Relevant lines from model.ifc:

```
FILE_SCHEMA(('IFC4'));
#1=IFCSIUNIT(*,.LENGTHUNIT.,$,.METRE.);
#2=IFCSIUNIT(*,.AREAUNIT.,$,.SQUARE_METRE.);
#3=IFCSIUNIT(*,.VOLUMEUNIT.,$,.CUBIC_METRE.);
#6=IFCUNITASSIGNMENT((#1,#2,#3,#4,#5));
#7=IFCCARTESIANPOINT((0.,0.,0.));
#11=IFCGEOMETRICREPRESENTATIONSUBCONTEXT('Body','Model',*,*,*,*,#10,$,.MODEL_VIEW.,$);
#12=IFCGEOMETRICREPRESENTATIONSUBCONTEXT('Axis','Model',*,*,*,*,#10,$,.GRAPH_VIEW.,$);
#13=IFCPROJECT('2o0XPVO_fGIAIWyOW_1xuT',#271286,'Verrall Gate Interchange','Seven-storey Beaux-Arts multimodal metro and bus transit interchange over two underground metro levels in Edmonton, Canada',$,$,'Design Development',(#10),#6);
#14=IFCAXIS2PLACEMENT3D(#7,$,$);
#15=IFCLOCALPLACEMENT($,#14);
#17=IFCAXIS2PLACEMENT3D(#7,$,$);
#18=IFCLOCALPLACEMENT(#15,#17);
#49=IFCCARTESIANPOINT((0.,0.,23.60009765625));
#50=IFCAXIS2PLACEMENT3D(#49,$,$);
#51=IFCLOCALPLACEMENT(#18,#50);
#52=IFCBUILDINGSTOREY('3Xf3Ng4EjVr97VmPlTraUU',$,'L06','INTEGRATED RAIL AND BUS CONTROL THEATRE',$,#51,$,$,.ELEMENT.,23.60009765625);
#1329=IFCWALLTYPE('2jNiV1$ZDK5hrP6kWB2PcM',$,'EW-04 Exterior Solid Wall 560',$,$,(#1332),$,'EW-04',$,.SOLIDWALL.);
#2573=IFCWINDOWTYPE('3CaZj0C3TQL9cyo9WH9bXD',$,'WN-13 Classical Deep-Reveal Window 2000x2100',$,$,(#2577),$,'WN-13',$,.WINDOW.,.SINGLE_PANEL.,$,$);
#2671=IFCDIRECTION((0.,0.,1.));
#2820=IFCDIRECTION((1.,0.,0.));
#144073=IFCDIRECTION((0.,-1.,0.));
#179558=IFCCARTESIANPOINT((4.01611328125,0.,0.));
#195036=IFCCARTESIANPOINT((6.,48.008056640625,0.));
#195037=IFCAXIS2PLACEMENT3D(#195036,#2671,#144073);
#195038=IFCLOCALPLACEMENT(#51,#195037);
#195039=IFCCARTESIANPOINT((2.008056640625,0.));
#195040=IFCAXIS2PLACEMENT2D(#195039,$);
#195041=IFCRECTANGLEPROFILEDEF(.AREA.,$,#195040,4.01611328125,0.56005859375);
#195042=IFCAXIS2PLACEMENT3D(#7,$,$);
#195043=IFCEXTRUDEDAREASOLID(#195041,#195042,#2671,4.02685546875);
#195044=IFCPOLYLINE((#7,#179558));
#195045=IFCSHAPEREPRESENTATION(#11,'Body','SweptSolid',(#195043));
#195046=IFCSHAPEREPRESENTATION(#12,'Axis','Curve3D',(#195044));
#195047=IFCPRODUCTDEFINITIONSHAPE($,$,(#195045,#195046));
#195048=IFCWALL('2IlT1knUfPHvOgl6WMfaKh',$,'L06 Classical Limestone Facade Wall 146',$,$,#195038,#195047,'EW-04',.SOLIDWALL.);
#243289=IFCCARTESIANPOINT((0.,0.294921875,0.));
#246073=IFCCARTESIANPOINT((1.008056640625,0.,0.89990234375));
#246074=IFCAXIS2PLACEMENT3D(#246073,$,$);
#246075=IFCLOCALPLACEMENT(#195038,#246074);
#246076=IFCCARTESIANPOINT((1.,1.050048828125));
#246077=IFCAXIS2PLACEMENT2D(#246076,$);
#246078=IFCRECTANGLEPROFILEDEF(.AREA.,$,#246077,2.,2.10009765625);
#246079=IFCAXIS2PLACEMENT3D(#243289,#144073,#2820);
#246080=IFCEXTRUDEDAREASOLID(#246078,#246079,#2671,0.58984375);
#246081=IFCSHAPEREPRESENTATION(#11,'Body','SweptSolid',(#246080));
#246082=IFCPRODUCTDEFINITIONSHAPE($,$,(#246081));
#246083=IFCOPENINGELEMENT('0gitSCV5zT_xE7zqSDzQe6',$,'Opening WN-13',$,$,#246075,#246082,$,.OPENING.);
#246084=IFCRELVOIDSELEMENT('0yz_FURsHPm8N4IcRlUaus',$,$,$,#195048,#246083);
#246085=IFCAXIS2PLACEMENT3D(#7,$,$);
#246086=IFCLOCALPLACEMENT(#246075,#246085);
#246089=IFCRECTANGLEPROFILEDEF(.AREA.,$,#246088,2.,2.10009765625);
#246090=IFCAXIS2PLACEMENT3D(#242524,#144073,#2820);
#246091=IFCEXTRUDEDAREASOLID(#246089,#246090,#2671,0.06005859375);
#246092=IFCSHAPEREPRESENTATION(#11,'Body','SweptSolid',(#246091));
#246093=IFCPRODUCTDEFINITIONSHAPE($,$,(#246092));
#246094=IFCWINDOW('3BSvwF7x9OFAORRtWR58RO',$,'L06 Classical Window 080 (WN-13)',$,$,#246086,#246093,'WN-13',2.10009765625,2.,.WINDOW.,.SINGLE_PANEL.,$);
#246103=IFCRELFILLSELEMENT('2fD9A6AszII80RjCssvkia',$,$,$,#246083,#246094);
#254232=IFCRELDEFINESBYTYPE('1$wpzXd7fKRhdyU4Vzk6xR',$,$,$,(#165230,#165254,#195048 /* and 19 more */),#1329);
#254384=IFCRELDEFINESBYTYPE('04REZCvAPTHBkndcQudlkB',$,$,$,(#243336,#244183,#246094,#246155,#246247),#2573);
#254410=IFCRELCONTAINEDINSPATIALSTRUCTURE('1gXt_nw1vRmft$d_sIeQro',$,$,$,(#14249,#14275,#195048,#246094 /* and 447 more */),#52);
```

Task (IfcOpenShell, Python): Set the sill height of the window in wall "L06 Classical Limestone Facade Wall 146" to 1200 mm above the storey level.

```python
import numpy as np
import ifcopenshell
import ifcopenshell.api.geometry
import ifcopenshell.geom
import ifcopenshell.util.element
import ifcopenshell.util.placement
import ifcopenshell.util.shape
import ifcopenshell.util.unit

model = ifcopenshell.open("model.ifc")
unit_scale = ifcopenshell.util.unit.calculate_unit_scale(model)

window = model.by_guid("3BSvwF7x9OFAORRtWR58RO")
opening = window.FillsVoids[0].RelatingOpeningElement
storey = ifcopenshell.util.element.get_container(window, ifc_class="IfcBuildingStorey")
level = ifcopenshell.util.placement.get_local_placement(storey.ObjectPlacement)[2, 3]

# The opening's origin need not be at the sill, so measure its lowest point.
shape = ifcopenshell.geom.create_shape(ifcopenshell.geom.settings(), opening)
bottom = ifcopenshell.util.shape.get_shape_bottom_elevation(shape, shape.geometry) / unit_scale
dz = level + 1.2 - bottom

shift = np.array([0.0, 0.0, dz])
# The window is placed relative to its opening, so it follows when the opening moves.
matrix = ifcopenshell.util.placement.get_local_placement(opening.ObjectPlacement)
matrix[:3, 3] += shift
ifcopenshell.api.geometry.edit_object_placement(
    model, product=opening, matrix=matrix, is_si=False, should_transform_children=True
)

print(f"moved by {dz * unit_scale:+.3f} m")

model.write("model_v2.ifc")
```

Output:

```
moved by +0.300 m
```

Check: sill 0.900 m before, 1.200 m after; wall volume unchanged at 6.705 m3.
